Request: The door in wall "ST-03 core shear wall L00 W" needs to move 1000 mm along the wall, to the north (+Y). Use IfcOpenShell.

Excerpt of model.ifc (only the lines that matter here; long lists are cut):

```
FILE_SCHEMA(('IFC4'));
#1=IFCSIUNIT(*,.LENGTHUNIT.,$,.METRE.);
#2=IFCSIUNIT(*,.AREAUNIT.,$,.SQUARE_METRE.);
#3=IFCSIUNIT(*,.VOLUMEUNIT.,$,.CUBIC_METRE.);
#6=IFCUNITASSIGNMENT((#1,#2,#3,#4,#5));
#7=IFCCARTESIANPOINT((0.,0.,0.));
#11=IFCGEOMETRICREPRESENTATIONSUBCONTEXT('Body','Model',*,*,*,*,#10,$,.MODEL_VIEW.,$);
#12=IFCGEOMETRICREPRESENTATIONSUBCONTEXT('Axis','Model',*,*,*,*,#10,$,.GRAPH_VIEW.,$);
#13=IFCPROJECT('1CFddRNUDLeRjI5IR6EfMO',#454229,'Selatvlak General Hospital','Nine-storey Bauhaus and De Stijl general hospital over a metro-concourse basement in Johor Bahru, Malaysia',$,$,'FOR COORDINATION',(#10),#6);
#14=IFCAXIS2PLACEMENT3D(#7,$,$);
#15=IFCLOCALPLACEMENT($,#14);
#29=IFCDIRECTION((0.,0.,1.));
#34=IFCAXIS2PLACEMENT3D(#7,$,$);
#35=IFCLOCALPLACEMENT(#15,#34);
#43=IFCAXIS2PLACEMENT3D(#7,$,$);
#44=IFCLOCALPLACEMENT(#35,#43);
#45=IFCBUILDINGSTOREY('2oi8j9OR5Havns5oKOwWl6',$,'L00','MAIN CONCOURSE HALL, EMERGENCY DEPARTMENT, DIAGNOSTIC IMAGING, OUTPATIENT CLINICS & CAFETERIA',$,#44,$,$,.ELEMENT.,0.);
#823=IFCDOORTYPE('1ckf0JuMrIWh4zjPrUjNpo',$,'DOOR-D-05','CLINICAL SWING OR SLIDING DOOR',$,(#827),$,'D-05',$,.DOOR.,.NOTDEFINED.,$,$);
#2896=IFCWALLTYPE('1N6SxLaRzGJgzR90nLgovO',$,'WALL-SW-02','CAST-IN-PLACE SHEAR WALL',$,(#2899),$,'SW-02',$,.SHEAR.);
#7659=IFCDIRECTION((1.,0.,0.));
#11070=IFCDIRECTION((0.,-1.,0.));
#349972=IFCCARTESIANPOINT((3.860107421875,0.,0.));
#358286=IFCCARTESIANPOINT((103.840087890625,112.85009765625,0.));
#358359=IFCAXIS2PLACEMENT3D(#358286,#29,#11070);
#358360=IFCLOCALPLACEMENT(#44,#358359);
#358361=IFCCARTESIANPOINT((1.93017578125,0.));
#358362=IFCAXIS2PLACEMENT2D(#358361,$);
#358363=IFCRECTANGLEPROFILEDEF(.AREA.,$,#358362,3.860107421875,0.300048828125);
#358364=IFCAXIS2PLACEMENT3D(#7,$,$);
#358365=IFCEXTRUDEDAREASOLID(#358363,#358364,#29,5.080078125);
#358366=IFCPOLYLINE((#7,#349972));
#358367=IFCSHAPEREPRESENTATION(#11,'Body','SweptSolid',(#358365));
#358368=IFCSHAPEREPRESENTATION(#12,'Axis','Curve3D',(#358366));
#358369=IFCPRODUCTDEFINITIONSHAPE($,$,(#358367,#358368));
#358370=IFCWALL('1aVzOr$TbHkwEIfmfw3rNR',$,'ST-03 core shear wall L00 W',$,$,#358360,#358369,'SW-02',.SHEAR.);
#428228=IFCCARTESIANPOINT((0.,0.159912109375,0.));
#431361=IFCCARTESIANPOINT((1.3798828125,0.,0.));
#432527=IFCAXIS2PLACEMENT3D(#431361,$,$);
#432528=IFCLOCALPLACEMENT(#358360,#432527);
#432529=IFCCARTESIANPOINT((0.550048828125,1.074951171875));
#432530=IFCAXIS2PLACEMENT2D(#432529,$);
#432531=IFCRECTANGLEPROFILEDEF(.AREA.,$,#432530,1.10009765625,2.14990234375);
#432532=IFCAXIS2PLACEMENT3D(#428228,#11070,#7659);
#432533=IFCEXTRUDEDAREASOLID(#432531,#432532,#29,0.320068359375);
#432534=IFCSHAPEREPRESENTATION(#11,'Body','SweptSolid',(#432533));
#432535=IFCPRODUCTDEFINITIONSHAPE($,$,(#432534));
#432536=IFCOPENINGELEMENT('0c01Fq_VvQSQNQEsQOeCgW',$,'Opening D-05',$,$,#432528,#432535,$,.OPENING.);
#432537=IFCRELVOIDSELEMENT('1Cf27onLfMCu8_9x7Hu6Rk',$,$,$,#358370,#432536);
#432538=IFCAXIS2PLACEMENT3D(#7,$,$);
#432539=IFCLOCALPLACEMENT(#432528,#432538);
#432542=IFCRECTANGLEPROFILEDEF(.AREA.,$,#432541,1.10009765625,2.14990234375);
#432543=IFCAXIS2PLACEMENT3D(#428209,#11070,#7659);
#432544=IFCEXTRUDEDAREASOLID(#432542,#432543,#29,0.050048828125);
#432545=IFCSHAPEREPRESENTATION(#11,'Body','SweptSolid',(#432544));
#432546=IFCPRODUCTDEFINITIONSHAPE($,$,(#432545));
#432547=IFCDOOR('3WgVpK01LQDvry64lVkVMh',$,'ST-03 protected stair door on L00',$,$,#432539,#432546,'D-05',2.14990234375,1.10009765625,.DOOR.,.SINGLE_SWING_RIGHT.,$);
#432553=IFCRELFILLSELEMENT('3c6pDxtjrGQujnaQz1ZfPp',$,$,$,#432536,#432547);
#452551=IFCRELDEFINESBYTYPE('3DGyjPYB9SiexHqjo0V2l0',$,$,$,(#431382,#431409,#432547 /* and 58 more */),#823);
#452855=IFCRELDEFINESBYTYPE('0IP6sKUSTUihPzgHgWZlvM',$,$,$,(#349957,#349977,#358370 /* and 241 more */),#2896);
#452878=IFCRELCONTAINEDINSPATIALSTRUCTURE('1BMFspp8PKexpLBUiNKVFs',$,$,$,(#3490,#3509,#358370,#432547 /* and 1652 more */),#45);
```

```python
import ifcopenshell
import ifcopenshell.api.geometry
import ifcopenshell.util.placement
import ifcopenshell.util.unit

model = ifcopenshell.open("model.ifc")
unit_scale = ifcopenshell.util.unit.calculate_unit_scale(model)

door = model.by_id(432547)
opening = door.FillsVoids[0].RelatingOpeningElement
wall = opening.VoidsElements[0].RelatingBuildingElement

wall_matrix = ifcopenshell.util.placement.get_local_placement(wall.ObjectPlacement)
shift = wall_matrix[:3, 0] * -1 / unit_scale
before = ifcopenshell.util.placement.get_local_placement(door.ObjectPlacement)[:3, 3].copy()

# The door is placed relative to its opening, so it follows when the opening moves.
matrix = ifcopenshell.util.placement.get_local_placement(opening.ObjectPlacement)
matrix[:3, 3] += shift
ifcopenshell.api.geometry.edit_object_placement(
    model, product=opening, matrix=matrix, is_si=False, should_transform_children=True
)

after = ifcopenshell.util.placement.get_local_placement(door.ObjectPlacement)[:3, 3]
print("door moved by", (after - before).round(3) + 0.0)

model.write("model-out.ifc")
```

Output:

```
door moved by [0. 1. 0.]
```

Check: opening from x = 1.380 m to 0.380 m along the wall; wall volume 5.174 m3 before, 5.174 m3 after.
